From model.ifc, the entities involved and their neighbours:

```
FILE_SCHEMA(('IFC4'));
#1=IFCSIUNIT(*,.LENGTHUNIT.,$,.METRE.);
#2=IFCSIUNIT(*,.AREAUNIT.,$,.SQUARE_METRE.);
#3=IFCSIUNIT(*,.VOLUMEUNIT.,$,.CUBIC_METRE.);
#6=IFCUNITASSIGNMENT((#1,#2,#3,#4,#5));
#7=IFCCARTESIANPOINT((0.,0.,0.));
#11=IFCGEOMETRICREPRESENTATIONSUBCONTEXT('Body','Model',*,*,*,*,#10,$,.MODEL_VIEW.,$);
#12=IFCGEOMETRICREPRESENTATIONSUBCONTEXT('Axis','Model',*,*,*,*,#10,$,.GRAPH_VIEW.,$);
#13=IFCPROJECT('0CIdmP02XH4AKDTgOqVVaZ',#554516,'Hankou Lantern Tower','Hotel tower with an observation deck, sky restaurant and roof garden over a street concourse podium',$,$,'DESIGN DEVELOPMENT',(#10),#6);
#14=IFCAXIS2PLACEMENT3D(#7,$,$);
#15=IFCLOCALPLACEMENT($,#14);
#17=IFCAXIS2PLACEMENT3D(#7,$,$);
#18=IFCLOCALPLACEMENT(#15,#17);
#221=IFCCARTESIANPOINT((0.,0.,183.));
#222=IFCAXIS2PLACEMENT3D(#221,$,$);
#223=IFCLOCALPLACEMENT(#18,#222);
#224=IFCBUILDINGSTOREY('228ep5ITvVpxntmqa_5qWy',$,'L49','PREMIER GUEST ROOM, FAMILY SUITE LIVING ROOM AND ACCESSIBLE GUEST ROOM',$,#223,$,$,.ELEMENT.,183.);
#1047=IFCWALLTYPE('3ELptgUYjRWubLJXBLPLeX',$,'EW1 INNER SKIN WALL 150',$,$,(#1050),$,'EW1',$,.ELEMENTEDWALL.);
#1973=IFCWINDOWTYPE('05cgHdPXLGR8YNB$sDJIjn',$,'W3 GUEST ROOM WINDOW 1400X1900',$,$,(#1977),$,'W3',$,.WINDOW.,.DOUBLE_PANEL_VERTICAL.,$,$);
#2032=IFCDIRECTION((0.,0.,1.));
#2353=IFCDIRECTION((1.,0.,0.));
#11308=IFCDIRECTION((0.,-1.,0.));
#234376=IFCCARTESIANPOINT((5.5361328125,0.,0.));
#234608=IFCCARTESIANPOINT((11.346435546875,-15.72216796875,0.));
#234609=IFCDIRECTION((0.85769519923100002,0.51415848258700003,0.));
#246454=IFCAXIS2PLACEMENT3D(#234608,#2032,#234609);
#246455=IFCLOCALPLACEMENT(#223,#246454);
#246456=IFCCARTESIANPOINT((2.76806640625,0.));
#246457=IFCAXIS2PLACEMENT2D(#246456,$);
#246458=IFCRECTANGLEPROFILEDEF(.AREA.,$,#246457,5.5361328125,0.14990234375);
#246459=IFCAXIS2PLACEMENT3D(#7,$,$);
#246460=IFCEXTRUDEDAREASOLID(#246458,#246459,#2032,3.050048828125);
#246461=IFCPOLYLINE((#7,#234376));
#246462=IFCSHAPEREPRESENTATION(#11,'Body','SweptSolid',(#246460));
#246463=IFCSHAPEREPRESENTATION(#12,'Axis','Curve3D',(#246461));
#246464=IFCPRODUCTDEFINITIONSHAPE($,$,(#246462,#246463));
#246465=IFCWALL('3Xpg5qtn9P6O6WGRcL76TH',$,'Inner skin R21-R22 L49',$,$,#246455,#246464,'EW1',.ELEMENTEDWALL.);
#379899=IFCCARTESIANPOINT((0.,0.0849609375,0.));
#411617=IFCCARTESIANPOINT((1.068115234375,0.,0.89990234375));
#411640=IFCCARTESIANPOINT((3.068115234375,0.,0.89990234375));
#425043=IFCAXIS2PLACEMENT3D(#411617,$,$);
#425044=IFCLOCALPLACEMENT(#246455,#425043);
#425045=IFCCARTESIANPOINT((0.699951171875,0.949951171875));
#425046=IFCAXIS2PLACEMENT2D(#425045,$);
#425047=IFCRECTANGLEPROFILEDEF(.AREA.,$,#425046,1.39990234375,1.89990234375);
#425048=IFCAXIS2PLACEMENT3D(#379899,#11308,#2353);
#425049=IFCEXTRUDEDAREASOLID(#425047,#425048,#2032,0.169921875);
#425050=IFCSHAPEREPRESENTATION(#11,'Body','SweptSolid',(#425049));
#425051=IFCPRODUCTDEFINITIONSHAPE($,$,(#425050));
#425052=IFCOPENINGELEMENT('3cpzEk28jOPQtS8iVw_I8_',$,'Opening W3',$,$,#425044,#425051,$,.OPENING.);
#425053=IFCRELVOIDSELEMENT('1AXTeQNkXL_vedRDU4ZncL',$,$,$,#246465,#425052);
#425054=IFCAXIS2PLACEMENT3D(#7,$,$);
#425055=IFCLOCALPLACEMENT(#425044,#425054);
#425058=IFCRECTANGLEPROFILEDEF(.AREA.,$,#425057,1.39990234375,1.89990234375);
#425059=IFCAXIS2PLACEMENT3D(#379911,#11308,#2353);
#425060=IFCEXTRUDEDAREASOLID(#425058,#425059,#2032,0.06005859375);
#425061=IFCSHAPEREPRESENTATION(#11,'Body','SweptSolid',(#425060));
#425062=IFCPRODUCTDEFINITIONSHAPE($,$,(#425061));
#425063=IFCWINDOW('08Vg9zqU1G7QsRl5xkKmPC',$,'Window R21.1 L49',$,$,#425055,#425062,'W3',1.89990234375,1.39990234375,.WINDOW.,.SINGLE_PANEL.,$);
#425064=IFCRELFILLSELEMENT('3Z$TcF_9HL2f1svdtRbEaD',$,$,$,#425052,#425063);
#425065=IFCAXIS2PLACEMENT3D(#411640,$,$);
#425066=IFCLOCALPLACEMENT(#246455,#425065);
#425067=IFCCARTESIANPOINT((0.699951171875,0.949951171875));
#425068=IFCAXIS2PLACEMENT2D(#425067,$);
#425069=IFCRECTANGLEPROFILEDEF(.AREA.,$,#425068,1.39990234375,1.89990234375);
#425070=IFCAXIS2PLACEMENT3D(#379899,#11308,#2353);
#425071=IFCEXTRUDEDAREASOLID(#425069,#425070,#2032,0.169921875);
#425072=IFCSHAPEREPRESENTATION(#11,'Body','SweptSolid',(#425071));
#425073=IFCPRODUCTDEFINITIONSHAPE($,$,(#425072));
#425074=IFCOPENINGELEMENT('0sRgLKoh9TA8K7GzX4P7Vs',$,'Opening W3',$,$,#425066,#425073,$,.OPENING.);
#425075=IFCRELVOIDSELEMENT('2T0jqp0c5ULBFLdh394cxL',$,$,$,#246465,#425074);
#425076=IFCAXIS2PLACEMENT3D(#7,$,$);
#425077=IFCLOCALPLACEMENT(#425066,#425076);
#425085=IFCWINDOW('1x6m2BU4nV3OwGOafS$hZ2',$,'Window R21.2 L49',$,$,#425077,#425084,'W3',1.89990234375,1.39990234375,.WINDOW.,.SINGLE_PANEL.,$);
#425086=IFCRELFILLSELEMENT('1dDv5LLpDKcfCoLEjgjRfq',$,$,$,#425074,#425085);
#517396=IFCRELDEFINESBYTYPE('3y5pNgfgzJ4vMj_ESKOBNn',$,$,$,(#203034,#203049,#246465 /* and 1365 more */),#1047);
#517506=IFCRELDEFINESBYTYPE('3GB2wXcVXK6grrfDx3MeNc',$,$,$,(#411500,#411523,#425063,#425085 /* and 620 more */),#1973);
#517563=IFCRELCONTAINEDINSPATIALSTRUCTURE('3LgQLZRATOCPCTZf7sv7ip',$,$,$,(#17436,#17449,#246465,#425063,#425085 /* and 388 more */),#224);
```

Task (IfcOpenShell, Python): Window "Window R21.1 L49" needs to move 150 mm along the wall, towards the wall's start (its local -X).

```python
import ifcopenshell
import ifcopenshell.api.geometry
import ifcopenshell.util.placement
import ifcopenshell.util.unit

model = ifcopenshell.open("model.ifc")
unit_scale = ifcopenshell.util.unit.calculate_unit_scale(model)

window = model.by_guid("08Vg9zqU1G7QsRl5xkKmPC")
opening = window.FillsVoids[0].RelatingOpeningElement
wall = opening.VoidsElements[0].RelatingBuildingElement

wall_matrix = ifcopenshell.util.placement.get_local_placement(wall.ObjectPlacement)
shift = wall_matrix[:3, 0] * -0.15 / unit_scale
before = ifcopenshell.util.placement.get_local_placement(window.ObjectPlacement)[:3, 3].copy()

# The window is placed relative to its opening, so it follows when the opening moves.
matrix = ifcopenshell.util.placement.get_local_placement(opening.ObjectPlacement)
matrix[:3, 3] += shift
ifcopenshell.api.geometry.edit_object_placement(
    model, product=opening, matrix=matrix, is_si=False, should_transform_children=True
)

after = ifcopenshell.util.placement.get_local_placement(window.ObjectPlacement)[:3, 3]
print("window moved by", (after - before).round(3) + 0.0)

model.write("model_updated.ifc")
```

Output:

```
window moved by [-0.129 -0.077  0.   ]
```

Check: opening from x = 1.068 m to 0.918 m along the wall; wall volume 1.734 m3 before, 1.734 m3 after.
